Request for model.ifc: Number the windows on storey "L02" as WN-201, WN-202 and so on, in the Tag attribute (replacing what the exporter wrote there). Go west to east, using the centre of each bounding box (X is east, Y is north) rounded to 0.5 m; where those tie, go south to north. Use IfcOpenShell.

First a look at what the model holds.

```python
import ifcopenshell
import ifcopenshell.util.element
import ifcopenshell.util.placement

model = ifcopenshell.open("model.ifc")
print(model.schema)
storey = next(s for s in model.by_type("IfcBuildingStorey") if s.Name == "L02")
windows = [e for e in ifcopenshell.util.element.get_decomposition(storey) if e.is_a("IfcWindow")]
for e in sorted(windows, key=lambda e: e.id()):
    origin = ifcopenshell.util.placement.get_local_placement(e.ObjectPlacement)[:3, 3]
    print(e.id(), e.Tag, e.Name, origin.round(2) + 0.0, sep=" | ")
```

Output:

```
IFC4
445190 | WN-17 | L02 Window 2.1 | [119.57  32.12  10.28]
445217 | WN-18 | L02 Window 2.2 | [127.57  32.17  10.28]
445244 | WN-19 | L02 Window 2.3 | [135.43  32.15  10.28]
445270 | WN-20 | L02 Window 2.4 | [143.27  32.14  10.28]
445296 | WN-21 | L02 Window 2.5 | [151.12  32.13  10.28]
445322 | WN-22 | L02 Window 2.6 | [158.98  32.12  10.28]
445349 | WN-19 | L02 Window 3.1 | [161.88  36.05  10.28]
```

```python
import ifcopenshell
import ifcopenshell.geom
import ifcopenshell.util.element
import ifcopenshell.util.shape

model = ifcopenshell.open("model.ifc")
settings = ifcopenshell.geom.settings()
settings.set("use-world-coords", True)


def centre(element):
    shape = ifcopenshell.geom.create_shape(settings, element)
    return ifcopenshell.util.shape.get_bbox_centroid(shape.geometry)


storey = next(s for s in model.by_type("IfcBuildingStorey") if s.Name == "L02")
windows = [e for e in ifcopenshell.util.element.get_decomposition(storey) if e.is_a("IfcWindow")]

# Insertion points can sit at a corner or the storey origin, so sort by the geometry (in metres).
centres = {e: centre(e) for e in windows}
windows.sort(key=lambda e: (round(centres[e][0] / 0.5), centres[e][1]))

for i, e in enumerate(windows, start=1):
    number = f"WN-2{i:02d}"
    e.Tag = number
    print(e.id(), number)

model.write("model_rev.ifc")
```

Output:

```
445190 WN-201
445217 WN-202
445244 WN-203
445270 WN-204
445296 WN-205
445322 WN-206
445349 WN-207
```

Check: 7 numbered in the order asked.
